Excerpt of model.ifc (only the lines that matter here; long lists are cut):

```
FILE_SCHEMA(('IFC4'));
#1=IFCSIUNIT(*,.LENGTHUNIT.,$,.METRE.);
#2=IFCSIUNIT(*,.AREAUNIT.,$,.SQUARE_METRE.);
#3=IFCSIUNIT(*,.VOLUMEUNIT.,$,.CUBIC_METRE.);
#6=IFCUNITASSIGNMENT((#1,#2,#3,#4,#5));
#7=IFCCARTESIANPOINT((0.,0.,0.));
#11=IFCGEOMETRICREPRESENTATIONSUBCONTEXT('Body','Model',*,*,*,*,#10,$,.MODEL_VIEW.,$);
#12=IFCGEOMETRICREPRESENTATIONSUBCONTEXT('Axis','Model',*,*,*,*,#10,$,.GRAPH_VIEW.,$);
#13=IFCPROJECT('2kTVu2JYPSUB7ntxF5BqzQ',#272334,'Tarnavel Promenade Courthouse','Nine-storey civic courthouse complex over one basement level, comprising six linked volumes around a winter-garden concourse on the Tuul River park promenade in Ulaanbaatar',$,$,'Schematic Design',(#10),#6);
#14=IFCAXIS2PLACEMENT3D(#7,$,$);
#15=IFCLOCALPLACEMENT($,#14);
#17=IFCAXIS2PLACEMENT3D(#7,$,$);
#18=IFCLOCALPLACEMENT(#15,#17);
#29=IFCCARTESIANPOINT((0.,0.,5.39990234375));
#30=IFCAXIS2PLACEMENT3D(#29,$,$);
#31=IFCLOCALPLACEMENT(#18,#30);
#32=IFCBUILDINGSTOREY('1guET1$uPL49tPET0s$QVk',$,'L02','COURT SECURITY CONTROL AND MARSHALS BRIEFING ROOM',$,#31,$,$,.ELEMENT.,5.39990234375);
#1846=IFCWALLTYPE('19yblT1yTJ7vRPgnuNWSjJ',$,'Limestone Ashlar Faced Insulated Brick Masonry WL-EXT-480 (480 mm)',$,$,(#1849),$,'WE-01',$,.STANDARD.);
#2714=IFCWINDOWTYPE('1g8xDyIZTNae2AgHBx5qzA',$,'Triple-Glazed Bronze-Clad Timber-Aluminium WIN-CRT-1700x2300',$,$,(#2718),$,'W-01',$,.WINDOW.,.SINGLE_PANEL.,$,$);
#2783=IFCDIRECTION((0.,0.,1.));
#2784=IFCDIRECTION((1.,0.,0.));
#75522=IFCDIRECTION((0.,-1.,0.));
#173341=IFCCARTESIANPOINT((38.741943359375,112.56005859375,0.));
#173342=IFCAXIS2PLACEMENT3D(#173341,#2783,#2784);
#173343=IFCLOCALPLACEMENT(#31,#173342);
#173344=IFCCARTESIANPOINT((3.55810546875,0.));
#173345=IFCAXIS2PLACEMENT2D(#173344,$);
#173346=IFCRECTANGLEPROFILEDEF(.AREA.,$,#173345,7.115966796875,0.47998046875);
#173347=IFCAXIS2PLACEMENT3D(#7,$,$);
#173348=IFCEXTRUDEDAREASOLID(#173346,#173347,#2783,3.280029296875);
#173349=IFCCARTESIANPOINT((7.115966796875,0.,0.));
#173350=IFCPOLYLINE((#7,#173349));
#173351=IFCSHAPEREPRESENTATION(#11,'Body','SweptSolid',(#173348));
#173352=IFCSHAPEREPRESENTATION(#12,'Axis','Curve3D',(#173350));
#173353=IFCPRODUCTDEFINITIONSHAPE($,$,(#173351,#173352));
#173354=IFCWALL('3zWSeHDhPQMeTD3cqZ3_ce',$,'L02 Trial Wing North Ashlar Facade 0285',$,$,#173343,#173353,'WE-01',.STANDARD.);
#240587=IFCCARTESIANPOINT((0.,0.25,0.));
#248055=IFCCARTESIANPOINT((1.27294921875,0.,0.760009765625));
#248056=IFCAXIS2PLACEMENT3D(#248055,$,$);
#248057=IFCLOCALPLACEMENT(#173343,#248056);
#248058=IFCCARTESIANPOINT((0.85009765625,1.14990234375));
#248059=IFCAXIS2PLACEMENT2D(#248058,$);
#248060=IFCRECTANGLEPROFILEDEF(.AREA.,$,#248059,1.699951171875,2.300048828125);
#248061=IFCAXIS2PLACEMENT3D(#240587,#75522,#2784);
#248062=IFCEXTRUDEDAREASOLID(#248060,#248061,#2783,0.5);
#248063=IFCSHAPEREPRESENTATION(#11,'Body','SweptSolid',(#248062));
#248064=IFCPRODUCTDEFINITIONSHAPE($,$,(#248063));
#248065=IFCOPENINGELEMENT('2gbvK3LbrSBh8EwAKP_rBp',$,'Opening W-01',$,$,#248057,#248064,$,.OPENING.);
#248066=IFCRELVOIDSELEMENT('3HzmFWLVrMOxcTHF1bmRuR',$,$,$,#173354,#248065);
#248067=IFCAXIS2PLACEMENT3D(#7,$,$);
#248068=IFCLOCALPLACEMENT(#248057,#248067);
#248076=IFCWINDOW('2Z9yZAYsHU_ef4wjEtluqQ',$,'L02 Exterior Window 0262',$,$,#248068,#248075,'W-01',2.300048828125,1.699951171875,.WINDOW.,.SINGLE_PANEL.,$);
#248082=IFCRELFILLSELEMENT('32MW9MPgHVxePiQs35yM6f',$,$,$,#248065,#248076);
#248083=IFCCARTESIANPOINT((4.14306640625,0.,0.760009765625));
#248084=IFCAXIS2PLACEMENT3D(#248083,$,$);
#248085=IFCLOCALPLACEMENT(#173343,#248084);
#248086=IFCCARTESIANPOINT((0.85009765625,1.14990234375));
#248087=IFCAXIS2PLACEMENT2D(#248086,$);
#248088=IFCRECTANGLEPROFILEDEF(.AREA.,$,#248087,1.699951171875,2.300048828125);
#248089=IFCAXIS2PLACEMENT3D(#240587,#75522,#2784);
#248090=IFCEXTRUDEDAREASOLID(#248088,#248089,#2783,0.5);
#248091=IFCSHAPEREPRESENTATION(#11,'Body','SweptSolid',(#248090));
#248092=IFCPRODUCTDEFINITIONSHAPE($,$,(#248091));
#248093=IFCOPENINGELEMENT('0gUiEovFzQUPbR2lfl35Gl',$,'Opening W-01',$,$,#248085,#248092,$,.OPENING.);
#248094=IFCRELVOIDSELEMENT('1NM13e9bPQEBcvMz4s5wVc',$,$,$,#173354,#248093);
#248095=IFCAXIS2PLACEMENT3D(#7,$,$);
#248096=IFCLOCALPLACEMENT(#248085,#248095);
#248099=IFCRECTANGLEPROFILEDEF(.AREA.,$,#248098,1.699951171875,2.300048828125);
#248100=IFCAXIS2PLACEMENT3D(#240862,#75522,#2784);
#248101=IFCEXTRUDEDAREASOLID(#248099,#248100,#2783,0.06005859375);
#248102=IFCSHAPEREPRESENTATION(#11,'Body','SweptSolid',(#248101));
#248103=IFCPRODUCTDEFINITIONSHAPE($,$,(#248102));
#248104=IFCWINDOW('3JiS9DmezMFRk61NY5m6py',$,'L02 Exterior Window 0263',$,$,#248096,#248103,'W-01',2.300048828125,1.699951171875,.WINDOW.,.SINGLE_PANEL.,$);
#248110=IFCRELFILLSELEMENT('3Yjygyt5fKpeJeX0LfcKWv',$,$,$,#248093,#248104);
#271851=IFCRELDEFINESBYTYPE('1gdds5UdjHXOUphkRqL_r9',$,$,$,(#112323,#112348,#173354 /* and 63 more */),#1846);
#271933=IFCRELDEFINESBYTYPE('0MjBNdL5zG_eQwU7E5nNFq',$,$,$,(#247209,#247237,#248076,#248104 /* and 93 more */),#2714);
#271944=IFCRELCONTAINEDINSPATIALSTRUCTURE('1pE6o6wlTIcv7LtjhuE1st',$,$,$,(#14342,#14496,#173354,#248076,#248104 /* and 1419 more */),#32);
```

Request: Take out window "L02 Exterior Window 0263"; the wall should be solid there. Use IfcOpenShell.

```python
import ifcopenshell
import ifcopenshell.api.feature
import ifcopenshell.api.root
import ifcopenshell.geom
import ifcopenshell.util.shape

model = ifcopenshell.open("model.ifc")
settings = ifcopenshell.geom.settings()


def volume(element):
    """Net volume in cubic metres, openings subtracted."""
    shape = ifcopenshell.geom.create_shape(settings, element)
    return ifcopenshell.util.shape.get_volume(shape.geometry)


window = model.by_id(248104)
opening = window.FillsVoids[0].RelatingOpeningElement
wall = opening.VoidsElements[0].RelatingBuildingElement
before = volume(wall)

ifcopenshell.api.root.remove_product(model, product=window)
ifcopenshell.api.feature.remove_feature(model, feature=opening)

after = volume(wall)

print(f"wall volume {before:.3f} -> {after:.3f} m3")

model.write("model_v2.ifc")
```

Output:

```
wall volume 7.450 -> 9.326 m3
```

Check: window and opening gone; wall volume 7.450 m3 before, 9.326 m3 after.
